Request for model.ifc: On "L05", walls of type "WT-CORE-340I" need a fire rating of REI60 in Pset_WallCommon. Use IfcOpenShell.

First a look at what the model holds.

```python
import ifcopenshell
import ifcopenshell.util.element

model = ifcopenshell.open("model.ifc")
print(model.schema)
storey = next(s for s in model.by_type("IfcBuildingStorey") if s.Name == "L05")
walls = [e for e in ifcopenshell.util.element.get_decomposition(storey) if e.is_a("IfcWall")]
seen = {}
for e in walls:
    element_type = ifcopenshell.util.element.get_type(e)
    key = (element_type.Name if element_type != e and element_type else None, ifcopenshell.util.element.get_pset(e, "Pset_WallCommon", "FireRating"))
    seen[key] = seen.get(key, 0) + 1
for (name, value), count in sorted(seen.items(), key=str):
    print(count, "x", name, "|", value)
```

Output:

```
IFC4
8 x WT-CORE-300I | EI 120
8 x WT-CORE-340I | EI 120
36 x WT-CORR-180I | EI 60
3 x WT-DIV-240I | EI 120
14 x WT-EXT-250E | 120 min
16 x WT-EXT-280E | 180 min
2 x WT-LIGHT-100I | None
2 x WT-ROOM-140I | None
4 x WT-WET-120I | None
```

```python
import ifcopenshell
import ifcopenshell.api.pset
import ifcopenshell.util.element

model = ifcopenshell.open("model.ifc")

storey = next(s for s in model.by_type("IfcBuildingStorey") if s.Name == "L05")
walls = [e for e in ifcopenshell.util.element.get_decomposition(storey) if e.is_a("IfcWall")]

count = 0
for e in walls:
    element_type = ifcopenshell.util.element.get_type(e)
    if element_type in (None, e) or element_type.Name != "WT-CORE-340I":
        continue
    # add_pset returns the element's existing set when there is one.
    pset = ifcopenshell.api.pset.add_pset(model, product=e, name="Pset_WallCommon")
    ifcopenshell.api.pset.edit_pset(model, pset=pset, properties={"FireRating": "REI60"})
    count += 1

print(count, "walls updated")

model.write("model_edited.ifc")
```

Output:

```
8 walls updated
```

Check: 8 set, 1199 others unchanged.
